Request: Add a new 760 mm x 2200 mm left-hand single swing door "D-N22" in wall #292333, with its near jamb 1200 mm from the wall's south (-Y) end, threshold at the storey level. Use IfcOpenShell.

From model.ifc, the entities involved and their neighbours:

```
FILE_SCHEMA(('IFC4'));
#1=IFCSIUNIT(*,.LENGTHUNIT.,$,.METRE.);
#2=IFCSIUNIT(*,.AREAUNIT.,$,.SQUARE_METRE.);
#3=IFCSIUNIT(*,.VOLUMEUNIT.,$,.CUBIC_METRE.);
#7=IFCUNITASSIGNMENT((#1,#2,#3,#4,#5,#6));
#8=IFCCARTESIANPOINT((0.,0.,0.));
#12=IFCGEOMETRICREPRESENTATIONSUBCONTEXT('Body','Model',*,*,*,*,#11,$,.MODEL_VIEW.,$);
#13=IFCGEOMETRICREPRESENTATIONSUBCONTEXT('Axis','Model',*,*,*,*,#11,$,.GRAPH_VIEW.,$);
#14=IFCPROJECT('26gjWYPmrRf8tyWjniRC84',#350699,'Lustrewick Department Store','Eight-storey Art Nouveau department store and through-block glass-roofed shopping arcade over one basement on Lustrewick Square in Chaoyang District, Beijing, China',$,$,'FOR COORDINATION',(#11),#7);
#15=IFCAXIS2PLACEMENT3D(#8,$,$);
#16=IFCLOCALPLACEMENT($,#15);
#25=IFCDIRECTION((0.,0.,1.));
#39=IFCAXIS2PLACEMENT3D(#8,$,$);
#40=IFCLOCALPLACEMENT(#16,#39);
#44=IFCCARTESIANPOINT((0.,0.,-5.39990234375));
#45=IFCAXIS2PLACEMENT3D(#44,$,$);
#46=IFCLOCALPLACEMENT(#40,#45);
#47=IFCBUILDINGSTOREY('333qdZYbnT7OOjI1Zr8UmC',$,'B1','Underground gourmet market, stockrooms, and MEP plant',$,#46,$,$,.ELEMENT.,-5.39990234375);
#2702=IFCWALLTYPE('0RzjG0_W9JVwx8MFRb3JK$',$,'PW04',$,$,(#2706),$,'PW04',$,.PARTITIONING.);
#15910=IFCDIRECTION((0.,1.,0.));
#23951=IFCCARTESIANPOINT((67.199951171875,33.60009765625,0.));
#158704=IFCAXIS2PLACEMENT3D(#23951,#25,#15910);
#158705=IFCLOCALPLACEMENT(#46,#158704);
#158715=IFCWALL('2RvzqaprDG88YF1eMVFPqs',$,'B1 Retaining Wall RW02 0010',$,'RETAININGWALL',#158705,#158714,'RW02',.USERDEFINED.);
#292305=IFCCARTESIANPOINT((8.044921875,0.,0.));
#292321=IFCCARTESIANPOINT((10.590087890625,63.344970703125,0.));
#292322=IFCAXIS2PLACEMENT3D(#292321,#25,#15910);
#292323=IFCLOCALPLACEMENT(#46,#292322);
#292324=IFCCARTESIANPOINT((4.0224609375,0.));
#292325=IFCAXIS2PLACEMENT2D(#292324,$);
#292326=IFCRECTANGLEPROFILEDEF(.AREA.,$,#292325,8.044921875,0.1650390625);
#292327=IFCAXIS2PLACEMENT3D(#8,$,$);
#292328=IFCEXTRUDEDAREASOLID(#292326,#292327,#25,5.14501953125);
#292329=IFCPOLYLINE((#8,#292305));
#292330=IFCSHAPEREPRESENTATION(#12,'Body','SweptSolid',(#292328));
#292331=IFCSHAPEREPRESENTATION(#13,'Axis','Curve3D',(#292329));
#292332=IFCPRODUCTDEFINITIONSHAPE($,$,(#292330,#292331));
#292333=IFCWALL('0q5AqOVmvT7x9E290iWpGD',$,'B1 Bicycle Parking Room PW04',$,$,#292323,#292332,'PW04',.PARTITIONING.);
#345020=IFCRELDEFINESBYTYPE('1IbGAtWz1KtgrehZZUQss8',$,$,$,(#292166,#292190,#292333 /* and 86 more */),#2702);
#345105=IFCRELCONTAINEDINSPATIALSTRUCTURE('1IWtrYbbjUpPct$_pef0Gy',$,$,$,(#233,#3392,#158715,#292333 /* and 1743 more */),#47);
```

```python
import numpy as np
import ifcopenshell
import ifcopenshell.api.feature
import ifcopenshell.api.geometry
import ifcopenshell.api.root
import ifcopenshell.api.spatial
import ifcopenshell.geom
import ifcopenshell.util.element
import ifcopenshell.util.placement
import ifcopenshell.util.representation
import ifcopenshell.util.shape
import ifcopenshell.util.unit

model = ifcopenshell.open("model.ifc")
unit_scale = ifcopenshell.util.unit.calculate_unit_scale(model)
settings = ifcopenshell.geom.settings()


def volume(element):
    """Net volume in cubic metres, openings subtracted."""
    shape = ifcopenshell.geom.create_shape(settings, element)
    return ifcopenshell.util.shape.get_volume(shape.geometry)


wall = model.by_id(292333)
storey = ifcopenshell.util.element.get_container(wall, ifc_class="IfcBuildingStorey")
context = ifcopenshell.util.representation.get_context(model, "Model", "Body", "MODEL_VIEW")
before = volume(wall)

width, height, from_end, sill = 0.76, 2.2, 1.2, 0.0  # metres

# The wall runs along its own X axis, and the end named is its -X end.
wall_shape = ifcopenshell.geom.create_shape(settings, wall)
x, y, z = ifcopenshell.util.shape.get_vertices(wall_shape.geometry).T
start = x.min() + from_end
face, thickness = float(y.min()), float(y.max() - y.min())
wall_matrix = ifcopenshell.util.placement.get_local_placement(wall.ObjectPlacement)
level = ifcopenshell.util.placement.get_local_placement(storey.ObjectPlacement)[2, 3]


def in_wall(x, y):
    """Placement at x, y metres in the wall's axes, at sill height."""
    matrix = wall_matrix.copy()
    matrix[:, 3] = wall_matrix @ np.array([x / unit_scale, y / unit_scale, 0.0, 1.0])
    matrix[2, 3] = level + sill / unit_scale
    return matrix


# Opening: a box that overshoots both wall faces by 50 mm.
opening = ifcopenshell.api.root.create_entity(model, ifc_class="IfcOpeningElement", predefined_type="OPENING")
box = ifcopenshell.api.geometry.add_wall_representation(
    model, context=context, length=width, height=height, thickness=thickness + 0.1
)
ifcopenshell.api.geometry.assign_representation(model, product=opening, representation=box)
ifcopenshell.api.geometry.edit_object_placement(model, product=opening, matrix=in_wall(start, face - 0.05), is_si=False)
ifcopenshell.api.feature.add_feature(model, feature=opening, element=wall)

door = ifcopenshell.api.root.create_entity(model, ifc_class="IfcDoor", name="D-N22", predefined_type="DOOR")
door.OverallWidth, door.OverallHeight = width / unit_scale, height / unit_scale
door.OperationType = "SINGLE_SWING_LEFT"
body = ifcopenshell.api.geometry.add_door_representation(
    model,
    context=context,
    overall_width=door.OverallWidth,
    overall_height=door.OverallHeight,
    operation_type="SINGLE_SWING_LEFT",
    lining_properties={"LiningDepth": thickness / unit_scale, "ThresholdDepth": thickness / unit_scale},
)
ifcopenshell.api.geometry.assign_representation(model, product=door, representation=body)
ifcopenshell.api.spatial.assign_container(model, products=[door], relating_structure=storey)
ifcopenshell.api.feature.add_filling(model, opening=opening, element=door)

# The lining spans the wall, so the door starts at the wall face.
ifcopenshell.api.geometry.edit_object_placement(model, product=door, matrix=in_wall(start, face), is_si=False)

after = volume(wall)

print(f"wall volume {before:.3f} -> {after:.3f} m3")

model.write("model_updated.ifc")
```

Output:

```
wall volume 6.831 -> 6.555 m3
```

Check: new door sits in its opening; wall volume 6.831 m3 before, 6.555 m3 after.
